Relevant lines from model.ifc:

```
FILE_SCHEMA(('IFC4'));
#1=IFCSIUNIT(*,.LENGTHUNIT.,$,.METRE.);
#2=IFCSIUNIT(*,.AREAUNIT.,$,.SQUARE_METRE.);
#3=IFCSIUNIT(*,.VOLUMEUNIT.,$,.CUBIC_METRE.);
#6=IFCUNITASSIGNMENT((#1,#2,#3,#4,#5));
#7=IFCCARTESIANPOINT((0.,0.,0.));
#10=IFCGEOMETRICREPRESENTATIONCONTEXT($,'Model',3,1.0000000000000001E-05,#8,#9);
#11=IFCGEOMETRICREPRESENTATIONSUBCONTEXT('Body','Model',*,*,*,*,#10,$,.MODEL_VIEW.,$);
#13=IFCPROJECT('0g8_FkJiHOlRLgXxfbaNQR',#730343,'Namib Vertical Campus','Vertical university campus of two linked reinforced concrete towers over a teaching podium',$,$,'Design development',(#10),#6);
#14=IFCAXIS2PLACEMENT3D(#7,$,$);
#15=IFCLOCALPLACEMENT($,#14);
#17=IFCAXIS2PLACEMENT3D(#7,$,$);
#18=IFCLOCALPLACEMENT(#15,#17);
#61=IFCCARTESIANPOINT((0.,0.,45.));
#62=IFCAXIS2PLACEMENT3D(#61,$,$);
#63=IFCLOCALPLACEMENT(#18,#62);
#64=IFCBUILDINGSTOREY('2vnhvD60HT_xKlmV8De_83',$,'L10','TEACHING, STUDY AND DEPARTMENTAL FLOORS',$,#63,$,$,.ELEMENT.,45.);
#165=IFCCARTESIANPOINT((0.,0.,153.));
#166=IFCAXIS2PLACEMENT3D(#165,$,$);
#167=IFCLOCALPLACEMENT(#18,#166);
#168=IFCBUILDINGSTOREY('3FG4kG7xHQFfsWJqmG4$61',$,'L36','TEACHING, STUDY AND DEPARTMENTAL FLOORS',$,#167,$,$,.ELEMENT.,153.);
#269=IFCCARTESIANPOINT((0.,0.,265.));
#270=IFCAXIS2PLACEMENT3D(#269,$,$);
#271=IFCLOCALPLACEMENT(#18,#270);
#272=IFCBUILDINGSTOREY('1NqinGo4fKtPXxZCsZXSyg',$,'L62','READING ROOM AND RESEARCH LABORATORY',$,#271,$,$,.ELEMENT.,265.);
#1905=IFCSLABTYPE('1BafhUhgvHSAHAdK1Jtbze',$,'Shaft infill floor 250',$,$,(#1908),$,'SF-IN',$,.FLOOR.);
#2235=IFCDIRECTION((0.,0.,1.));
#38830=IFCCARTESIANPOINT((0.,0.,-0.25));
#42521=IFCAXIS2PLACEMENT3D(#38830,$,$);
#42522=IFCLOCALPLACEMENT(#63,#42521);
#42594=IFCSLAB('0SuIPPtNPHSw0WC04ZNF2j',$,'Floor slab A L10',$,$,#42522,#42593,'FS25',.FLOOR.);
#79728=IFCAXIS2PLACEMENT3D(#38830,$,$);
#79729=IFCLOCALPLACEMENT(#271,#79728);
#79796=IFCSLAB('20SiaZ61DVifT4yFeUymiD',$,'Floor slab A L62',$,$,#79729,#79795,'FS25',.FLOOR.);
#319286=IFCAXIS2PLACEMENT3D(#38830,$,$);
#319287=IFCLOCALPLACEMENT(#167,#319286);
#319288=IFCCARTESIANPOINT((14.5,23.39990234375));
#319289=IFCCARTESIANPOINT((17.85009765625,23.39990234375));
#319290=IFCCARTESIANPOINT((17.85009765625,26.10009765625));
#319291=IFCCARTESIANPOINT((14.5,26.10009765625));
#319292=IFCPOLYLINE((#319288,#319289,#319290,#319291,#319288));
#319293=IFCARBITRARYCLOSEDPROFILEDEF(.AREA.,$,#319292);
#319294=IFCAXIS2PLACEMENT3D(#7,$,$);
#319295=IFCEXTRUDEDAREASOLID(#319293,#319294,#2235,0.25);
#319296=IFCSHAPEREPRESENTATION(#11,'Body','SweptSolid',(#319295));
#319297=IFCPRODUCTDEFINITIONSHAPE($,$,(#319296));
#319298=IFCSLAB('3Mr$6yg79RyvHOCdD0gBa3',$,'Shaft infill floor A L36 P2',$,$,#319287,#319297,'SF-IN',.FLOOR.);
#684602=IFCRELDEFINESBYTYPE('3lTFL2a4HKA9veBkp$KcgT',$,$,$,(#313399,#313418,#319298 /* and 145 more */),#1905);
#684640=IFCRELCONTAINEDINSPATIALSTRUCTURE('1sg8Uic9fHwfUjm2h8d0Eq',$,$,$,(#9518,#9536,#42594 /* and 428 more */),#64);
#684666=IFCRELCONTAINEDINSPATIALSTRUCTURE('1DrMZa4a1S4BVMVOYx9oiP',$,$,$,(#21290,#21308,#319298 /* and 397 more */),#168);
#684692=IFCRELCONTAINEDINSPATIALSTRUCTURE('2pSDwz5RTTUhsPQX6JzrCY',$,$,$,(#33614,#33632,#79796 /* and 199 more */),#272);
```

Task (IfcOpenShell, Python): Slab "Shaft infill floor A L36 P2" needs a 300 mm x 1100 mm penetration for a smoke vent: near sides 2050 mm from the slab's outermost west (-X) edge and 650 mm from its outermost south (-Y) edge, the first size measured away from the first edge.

```python
import numpy as np
import ifcopenshell
import ifcopenshell.api.feature
import ifcopenshell.api.geometry
import ifcopenshell.api.root
import ifcopenshell.geom
import ifcopenshell.util.placement
import ifcopenshell.util.representation
import ifcopenshell.util.shape
import ifcopenshell.util.unit

model = ifcopenshell.open("model.ifc")
unit_scale = ifcopenshell.util.unit.calculate_unit_scale(model)
settings = ifcopenshell.geom.settings()


def volume(element):
    """Net volume in cubic metres, openings subtracted."""
    shape = ifcopenshell.geom.create_shape(settings, element)
    return ifcopenshell.util.shape.get_volume(shape.geometry)


slab = model.by_id(319298)
before = volume(slab)

# Extent in the slab's own axes, in metres. The edges named are its -X and -Y sides.
slab_shape = ifcopenshell.geom.create_shape(settings, slab)
vertices = ifcopenshell.util.shape.get_vertices(slab_shape.geometry)
x_min, y_min, bottom = vertices.min(axis=0)
top = vertices[:, 2].max()

opening = ifcopenshell.api.root.create_entity(model, ifc_class="IfcOpeningElement", name="Smoke vent opening", predefined_type="OPENING")
context = ifcopenshell.util.representation.get_context(model, "Model", "Body", "MODEL_VIEW")
width, depth = 0.3, 1.1
outline = [(0.0, 0.0), (width, 0.0), (width, depth), (0.0, depth), (0.0, 0.0)]
# Overshoot both faces by 50 mm so the cut is clean.
shape = ifcopenshell.api.geometry.add_slab_representation(
    model, context=context, depth=top - bottom + 0.1, polyline=outline
)
ifcopenshell.api.geometry.assign_representation(model, product=opening, representation=shape)

matrix = ifcopenshell.util.placement.get_local_placement(slab.ObjectPlacement)
matrix[:, 3] = matrix @ np.append(np.array([x_min + 2.05, y_min + 0.65, bottom - 0.05]) / unit_scale, 1.0)
ifcopenshell.api.geometry.edit_object_placement(model, product=opening, matrix=matrix, is_si=False)
ifcopenshell.api.feature.add_feature(model, feature=opening, element=slab)

after = volume(slab)

print(f"slab volume {before:.3f} -> {after:.3f} m3")

model.write("model_rev.ifc")
```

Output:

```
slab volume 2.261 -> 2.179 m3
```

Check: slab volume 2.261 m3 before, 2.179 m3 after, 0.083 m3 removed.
